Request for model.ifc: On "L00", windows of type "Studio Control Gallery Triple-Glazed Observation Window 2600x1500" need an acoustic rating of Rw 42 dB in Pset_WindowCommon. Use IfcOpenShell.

First a look at what the model holds.

```python
import ifcopenshell
import ifcopenshell.util.element

model = ifcopenshell.open("model.ifc")
print(model.schema)
storey = next(s for s in model.by_type("IfcBuildingStorey") if s.Name == "L00")
windows = [e for e in ifcopenshell.util.element.get_decomposition(storey) if e.is_a("IfcWindow")]
seen = {}
for e in windows:
    element_type = ifcopenshell.util.element.get_type(e)
    key = (element_type.Name if element_type != e and element_type else None, ifcopenshell.util.element.get_pset(e, "Pset_WindowCommon", "AcousticRating"))
    seen[key] = seen.get(key, 0) + 1
for (name, value), count in sorted(seen.items(), key=str):
    print(count, "x", name, "|", value)
```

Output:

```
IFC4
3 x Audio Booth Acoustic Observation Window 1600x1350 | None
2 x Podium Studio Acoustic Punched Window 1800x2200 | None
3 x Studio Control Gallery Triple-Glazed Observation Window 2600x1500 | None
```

```python
import ifcopenshell
import ifcopenshell.api.pset
import ifcopenshell.util.element

model = ifcopenshell.open("model.ifc")

storey = next(s for s in model.by_type("IfcBuildingStorey") if s.Name == "L00")
windows = [e for e in ifcopenshell.util.element.get_decomposition(storey) if e.is_a("IfcWindow")]

count = 0
for e in windows:
    element_type = ifcopenshell.util.element.get_type(e)
    if element_type in (None, e) or element_type.Name != "Studio Control Gallery Triple-Glazed Observation Window 2600x1500":
        continue
    found = ifcopenshell.util.element.get_pset(e, "Pset_WindowCommon", should_inherit=False)
    if found:
        pset = model.by_id(found["id"])
        if len(ifcopenshell.util.element.get_elements_by_pset(pset)) > 1:
            pset = ifcopenshell.api.pset.unshare_pset(model, products=[e], pset=pset)[0]
    else:
        pset = ifcopenshell.api.pset.add_pset(model, product=e, name="Pset_WindowCommon")
    ifcopenshell.api.pset.edit_pset(model, pset=pset, properties={"AcousticRating": "Rw 42 dB"})
    count += 1

print(count, "windows updated")

model.write("model_v2.ifc")
```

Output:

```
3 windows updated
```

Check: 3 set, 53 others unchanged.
